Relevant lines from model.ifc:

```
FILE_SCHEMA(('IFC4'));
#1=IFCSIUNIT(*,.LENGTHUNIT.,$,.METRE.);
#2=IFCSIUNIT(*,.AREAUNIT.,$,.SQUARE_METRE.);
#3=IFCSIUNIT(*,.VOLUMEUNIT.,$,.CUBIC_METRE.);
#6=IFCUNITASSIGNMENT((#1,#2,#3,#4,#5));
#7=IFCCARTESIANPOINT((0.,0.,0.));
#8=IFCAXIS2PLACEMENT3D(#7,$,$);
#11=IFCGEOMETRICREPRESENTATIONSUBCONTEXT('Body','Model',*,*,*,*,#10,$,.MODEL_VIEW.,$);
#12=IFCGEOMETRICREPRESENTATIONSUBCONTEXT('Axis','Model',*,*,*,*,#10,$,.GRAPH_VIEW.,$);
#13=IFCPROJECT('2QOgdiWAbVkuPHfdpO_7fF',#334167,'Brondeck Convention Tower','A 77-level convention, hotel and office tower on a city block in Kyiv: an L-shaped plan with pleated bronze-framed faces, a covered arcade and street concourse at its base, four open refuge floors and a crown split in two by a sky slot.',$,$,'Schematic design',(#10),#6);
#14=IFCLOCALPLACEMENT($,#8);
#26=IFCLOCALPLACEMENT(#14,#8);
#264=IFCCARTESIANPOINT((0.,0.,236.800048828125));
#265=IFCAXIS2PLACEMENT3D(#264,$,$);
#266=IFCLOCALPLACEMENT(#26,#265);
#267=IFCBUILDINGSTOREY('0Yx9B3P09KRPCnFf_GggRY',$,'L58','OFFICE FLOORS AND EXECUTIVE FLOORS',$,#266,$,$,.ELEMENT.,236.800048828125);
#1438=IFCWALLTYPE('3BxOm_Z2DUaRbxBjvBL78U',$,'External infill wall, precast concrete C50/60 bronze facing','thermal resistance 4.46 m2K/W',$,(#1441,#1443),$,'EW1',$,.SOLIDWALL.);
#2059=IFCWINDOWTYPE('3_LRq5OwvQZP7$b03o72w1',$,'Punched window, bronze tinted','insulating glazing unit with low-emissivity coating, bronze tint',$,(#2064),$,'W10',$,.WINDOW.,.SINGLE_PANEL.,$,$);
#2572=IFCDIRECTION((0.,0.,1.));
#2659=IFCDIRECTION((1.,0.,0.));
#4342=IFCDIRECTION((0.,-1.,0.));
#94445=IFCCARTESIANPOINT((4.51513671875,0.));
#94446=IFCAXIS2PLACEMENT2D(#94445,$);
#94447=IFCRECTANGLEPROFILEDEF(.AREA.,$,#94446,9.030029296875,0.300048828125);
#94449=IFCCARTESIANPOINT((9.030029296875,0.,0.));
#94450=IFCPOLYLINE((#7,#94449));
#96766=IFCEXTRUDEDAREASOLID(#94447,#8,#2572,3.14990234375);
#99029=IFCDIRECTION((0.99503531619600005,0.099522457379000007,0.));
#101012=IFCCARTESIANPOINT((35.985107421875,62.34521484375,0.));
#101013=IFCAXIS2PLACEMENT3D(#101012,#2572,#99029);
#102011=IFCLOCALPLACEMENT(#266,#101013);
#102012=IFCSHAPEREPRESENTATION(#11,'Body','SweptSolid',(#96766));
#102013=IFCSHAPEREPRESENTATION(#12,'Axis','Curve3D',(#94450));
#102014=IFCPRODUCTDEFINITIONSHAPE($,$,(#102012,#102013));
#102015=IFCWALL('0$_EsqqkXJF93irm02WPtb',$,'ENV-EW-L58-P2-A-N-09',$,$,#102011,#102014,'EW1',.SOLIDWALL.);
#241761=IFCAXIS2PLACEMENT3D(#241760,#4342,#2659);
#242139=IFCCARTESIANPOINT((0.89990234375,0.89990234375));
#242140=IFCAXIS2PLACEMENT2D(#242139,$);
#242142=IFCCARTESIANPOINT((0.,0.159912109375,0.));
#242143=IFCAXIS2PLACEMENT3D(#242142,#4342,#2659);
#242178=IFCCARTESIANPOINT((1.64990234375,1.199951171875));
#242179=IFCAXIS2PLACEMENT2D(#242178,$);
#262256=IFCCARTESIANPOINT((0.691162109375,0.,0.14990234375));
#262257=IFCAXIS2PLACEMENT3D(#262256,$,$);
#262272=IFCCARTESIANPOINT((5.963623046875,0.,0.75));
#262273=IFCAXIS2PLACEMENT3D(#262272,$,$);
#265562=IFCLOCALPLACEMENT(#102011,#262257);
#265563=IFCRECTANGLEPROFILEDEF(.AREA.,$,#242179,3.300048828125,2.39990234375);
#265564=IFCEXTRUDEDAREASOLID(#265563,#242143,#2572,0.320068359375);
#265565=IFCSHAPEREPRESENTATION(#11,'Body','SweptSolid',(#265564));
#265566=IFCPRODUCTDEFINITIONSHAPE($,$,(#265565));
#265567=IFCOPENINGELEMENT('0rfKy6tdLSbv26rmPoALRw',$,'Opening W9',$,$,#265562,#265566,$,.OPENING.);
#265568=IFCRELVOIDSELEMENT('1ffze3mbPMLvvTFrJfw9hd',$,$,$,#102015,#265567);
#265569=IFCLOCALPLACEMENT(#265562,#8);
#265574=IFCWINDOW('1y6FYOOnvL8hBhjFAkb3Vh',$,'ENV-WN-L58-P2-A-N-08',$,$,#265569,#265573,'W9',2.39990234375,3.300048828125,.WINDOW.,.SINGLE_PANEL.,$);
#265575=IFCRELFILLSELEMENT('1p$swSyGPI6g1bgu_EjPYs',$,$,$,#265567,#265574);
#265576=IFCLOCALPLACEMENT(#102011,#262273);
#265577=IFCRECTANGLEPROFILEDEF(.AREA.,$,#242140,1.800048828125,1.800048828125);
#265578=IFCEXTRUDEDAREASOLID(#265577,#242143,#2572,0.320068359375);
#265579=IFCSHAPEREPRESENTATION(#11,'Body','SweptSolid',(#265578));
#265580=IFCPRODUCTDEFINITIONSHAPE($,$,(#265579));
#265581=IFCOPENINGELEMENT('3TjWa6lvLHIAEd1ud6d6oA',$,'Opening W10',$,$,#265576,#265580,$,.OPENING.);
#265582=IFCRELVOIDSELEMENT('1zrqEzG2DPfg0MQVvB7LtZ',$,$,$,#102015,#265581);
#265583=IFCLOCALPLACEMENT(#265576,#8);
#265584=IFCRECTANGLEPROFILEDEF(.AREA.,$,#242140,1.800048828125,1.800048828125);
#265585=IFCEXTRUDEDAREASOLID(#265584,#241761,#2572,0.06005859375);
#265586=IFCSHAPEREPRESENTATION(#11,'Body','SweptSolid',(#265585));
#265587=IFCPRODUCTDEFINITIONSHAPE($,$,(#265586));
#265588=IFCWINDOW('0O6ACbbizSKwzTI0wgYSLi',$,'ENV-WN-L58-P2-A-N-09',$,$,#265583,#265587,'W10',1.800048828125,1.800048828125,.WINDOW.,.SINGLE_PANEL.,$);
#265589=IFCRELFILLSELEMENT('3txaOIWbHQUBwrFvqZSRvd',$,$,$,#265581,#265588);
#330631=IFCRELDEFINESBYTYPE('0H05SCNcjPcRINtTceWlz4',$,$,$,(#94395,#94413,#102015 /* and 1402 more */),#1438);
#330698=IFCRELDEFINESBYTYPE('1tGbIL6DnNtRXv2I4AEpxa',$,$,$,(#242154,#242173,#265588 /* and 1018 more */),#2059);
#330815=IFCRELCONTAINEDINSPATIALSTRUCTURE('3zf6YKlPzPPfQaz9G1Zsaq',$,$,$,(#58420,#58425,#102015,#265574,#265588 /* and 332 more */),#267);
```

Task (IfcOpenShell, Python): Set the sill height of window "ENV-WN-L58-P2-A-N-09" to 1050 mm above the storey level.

```python
import numpy as np
import ifcopenshell
import ifcopenshell.api.geometry
import ifcopenshell.geom
import ifcopenshell.util.element
import ifcopenshell.util.placement
import ifcopenshell.util.shape
import ifcopenshell.util.unit

model = ifcopenshell.open("model.ifc")
unit_scale = ifcopenshell.util.unit.calculate_unit_scale(model)

window = model.by_id(265588)
opening = window.FillsVoids[0].RelatingOpeningElement
storey = ifcopenshell.util.element.get_container(window, ifc_class="IfcBuildingStorey")
level = ifcopenshell.util.placement.get_local_placement(storey.ObjectPlacement)[2, 3]

# The opening's origin need not be at the sill, so measure its lowest point.
shape = ifcopenshell.geom.create_shape(ifcopenshell.geom.settings(), opening)
bottom = ifcopenshell.util.shape.get_shape_bottom_elevation(shape, shape.geometry) / unit_scale
dz = level + 1.05 - bottom

shift = np.array([0.0, 0.0, dz])
# The window is placed relative to its opening, so it follows when the opening moves.
matrix = ifcopenshell.util.placement.get_local_placement(opening.ObjectPlacement)
matrix[:3, 3] += shift
ifcopenshell.api.geometry.edit_object_placement(
    model, product=opening, matrix=matrix, is_si=False, should_transform_children=True
)

print(f"moved by {dz * unit_scale:+.3f} m")

model.write("model_rev.ifc")
```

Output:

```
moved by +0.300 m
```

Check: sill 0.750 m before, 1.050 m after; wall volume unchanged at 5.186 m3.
